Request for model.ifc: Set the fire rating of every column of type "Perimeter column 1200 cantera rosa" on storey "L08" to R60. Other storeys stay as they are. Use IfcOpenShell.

First a look at what the model holds.

```python
import ifcopenshell
import ifcopenshell.util.element

model = ifcopenshell.open("model.ifc")
print(model.schema)
storey = next(s for s in model.by_type("IfcBuildingStorey") if s.Name == "L08")
columns = [e for e in ifcopenshell.util.element.get_decomposition(storey) if e.is_a("IfcColumn")]
seen = {}
for e in columns:
    element_type = ifcopenshell.util.element.get_type(e)
    key = (element_type.Name if element_type != e and element_type else None, ifcopenshell.util.element.get_pset(e, "Pset_ColumnCommon", "FireRating"))
    seen[key] = seen.get(key, 0) + 1
for (name, value), count in sorted(seen.items(), key=str):
    print(count, "x", name, "|", value)
```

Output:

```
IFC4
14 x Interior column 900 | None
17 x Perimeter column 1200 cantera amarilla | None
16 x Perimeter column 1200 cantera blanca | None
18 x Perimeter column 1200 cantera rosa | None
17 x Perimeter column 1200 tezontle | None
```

```python
import ifcopenshell
import ifcopenshell.api.pset
import ifcopenshell.util.element

model = ifcopenshell.open("model.ifc")

storey = next(s for s in model.by_type("IfcBuildingStorey") if s.Name == "L08")
columns = [e for e in ifcopenshell.util.element.get_decomposition(storey) if e.is_a("IfcColumn")]

count = 0
for e in columns:
    element_type = ifcopenshell.util.element.get_type(e)
    if element_type in (None, e) or element_type.Name != "Perimeter column 1200 cantera rosa":
        continue
    found = ifcopenshell.util.element.get_pset(e, "Pset_ColumnCommon", should_inherit=False)
    if found:
        pset = model.by_id(found["id"])
        if len(ifcopenshell.util.element.get_elements_by_pset(pset)) > 1:
            pset = ifcopenshell.api.pset.unshare_pset(model, products=[e], pset=pset)[0]
    else:
        pset = ifcopenshell.api.pset.add_pset(model, product=e, name="Pset_ColumnCommon")
    ifcopenshell.api.pset.edit_pset(model, pset=pset, properties={"FireRating": "R60"})
    count += 1

print(count, "columns updated")

model.write("model_edited.ifc")
```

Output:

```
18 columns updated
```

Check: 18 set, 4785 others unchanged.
